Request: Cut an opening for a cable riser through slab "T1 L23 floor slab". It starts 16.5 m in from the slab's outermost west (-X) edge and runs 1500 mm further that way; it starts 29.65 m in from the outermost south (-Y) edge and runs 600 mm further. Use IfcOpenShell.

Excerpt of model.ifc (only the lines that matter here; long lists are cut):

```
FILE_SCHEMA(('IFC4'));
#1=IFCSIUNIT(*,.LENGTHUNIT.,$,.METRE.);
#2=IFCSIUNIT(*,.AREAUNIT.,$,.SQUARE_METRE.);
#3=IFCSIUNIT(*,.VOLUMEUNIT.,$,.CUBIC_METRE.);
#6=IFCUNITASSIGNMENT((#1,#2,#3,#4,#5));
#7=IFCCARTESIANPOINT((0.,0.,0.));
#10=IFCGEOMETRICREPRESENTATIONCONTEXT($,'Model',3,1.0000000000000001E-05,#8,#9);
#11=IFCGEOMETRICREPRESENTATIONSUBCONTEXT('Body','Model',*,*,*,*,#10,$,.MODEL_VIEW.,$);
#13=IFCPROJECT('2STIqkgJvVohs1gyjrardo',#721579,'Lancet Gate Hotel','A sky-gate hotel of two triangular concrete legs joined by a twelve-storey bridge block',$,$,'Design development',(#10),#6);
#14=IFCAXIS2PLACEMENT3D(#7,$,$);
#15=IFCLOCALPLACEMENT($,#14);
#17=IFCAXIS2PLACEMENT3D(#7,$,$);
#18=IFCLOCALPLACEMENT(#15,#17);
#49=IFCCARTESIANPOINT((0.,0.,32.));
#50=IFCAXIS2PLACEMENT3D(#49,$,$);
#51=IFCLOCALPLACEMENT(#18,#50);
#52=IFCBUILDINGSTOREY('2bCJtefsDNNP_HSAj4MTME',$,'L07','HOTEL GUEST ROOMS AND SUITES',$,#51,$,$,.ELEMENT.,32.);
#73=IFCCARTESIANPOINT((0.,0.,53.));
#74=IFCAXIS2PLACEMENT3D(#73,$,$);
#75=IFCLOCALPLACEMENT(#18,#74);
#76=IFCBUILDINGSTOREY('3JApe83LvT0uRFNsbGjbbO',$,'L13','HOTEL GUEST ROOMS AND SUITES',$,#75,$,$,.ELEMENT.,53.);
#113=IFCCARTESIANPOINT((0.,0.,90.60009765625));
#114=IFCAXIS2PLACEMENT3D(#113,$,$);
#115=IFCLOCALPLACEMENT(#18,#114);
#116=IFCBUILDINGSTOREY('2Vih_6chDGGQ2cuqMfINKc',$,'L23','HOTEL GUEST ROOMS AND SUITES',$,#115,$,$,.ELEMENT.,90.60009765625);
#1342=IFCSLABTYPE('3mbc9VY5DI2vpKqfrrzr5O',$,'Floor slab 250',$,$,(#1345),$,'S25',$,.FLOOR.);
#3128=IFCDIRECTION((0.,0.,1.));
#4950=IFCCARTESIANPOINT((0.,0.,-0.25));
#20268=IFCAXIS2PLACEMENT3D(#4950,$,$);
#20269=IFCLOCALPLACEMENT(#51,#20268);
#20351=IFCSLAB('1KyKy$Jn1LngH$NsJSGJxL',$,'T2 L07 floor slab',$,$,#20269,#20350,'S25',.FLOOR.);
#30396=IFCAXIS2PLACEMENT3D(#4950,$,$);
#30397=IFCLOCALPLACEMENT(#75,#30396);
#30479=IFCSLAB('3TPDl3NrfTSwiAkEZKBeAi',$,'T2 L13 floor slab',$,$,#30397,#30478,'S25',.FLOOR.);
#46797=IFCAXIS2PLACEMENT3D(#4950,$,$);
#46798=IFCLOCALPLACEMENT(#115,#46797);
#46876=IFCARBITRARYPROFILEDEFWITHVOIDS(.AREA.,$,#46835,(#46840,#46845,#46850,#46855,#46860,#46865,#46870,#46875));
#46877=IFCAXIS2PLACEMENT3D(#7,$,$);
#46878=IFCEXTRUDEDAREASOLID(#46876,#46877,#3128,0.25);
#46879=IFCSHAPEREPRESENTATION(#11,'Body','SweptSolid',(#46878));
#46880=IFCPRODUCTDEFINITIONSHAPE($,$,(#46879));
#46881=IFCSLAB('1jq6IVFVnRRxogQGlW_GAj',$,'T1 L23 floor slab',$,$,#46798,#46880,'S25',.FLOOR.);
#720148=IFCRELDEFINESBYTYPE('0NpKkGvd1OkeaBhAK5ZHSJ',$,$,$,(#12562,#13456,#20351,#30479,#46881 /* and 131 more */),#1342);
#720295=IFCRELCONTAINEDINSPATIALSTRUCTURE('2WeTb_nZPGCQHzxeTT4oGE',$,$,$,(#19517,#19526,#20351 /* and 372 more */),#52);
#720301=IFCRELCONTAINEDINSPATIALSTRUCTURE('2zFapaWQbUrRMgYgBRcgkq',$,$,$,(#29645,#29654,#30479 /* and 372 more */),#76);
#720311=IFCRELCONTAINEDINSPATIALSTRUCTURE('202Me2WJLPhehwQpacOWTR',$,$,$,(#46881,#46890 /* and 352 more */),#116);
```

```python
import numpy as np
import ifcopenshell
import ifcopenshell.api.feature
import ifcopenshell.api.geometry
import ifcopenshell.api.root
import ifcopenshell.geom
import ifcopenshell.util.placement
import ifcopenshell.util.representation
import ifcopenshell.util.shape
import ifcopenshell.util.unit

model = ifcopenshell.open("model.ifc")
unit_scale = ifcopenshell.util.unit.calculate_unit_scale(model)
settings = ifcopenshell.geom.settings()


def volume(element):
    """Net volume in cubic metres, openings subtracted."""
    shape = ifcopenshell.geom.create_shape(settings, element)
    return ifcopenshell.util.shape.get_volume(shape.geometry)


slab = model.by_guid("1jq6IVFVnRRxogQGlW_GAj")
before = volume(slab)

# Extent in the slab's own axes, in metres. The edges named are its -X and -Y sides.
slab_shape = ifcopenshell.geom.create_shape(settings, slab)
vertices = ifcopenshell.util.shape.get_vertices(slab_shape.geometry)
x_min, y_min, bottom = vertices.min(axis=0)
top = vertices[:, 2].max()

opening = ifcopenshell.api.root.create_entity(model, ifc_class="IfcOpeningElement", name="Cable riser opening", predefined_type="OPENING")
context = ifcopenshell.util.representation.get_context(model, "Model", "Body", "MODEL_VIEW")
width, depth = 1.5, 0.6
outline = [(0.0, 0.0), (width, 0.0), (width, depth), (0.0, depth), (0.0, 0.0)]
# Overshoot both faces by 50 mm so the cut is clean.
shape = ifcopenshell.api.geometry.add_slab_representation(
    model, context=context, depth=top - bottom + 0.1, polyline=outline
)
ifcopenshell.api.geometry.assign_representation(model, product=opening, representation=shape)

matrix = ifcopenshell.util.placement.get_local_placement(slab.ObjectPlacement)
matrix[:, 3] = matrix @ np.append(np.array([x_min + 16.5, y_min + 29.65, bottom - 0.05]) / unit_scale, 1.0)
ifcopenshell.api.geometry.edit_object_placement(model, product=opening, matrix=matrix, is_si=False)
ifcopenshell.api.feature.add_feature(model, feature=opening, element=slab)

after = volume(slab)

print(f"slab volume {before:.3f} -> {after:.3f} m3")

model.write("model_edited.ifc")
```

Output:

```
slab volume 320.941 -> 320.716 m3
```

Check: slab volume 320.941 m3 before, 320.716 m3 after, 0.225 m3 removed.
